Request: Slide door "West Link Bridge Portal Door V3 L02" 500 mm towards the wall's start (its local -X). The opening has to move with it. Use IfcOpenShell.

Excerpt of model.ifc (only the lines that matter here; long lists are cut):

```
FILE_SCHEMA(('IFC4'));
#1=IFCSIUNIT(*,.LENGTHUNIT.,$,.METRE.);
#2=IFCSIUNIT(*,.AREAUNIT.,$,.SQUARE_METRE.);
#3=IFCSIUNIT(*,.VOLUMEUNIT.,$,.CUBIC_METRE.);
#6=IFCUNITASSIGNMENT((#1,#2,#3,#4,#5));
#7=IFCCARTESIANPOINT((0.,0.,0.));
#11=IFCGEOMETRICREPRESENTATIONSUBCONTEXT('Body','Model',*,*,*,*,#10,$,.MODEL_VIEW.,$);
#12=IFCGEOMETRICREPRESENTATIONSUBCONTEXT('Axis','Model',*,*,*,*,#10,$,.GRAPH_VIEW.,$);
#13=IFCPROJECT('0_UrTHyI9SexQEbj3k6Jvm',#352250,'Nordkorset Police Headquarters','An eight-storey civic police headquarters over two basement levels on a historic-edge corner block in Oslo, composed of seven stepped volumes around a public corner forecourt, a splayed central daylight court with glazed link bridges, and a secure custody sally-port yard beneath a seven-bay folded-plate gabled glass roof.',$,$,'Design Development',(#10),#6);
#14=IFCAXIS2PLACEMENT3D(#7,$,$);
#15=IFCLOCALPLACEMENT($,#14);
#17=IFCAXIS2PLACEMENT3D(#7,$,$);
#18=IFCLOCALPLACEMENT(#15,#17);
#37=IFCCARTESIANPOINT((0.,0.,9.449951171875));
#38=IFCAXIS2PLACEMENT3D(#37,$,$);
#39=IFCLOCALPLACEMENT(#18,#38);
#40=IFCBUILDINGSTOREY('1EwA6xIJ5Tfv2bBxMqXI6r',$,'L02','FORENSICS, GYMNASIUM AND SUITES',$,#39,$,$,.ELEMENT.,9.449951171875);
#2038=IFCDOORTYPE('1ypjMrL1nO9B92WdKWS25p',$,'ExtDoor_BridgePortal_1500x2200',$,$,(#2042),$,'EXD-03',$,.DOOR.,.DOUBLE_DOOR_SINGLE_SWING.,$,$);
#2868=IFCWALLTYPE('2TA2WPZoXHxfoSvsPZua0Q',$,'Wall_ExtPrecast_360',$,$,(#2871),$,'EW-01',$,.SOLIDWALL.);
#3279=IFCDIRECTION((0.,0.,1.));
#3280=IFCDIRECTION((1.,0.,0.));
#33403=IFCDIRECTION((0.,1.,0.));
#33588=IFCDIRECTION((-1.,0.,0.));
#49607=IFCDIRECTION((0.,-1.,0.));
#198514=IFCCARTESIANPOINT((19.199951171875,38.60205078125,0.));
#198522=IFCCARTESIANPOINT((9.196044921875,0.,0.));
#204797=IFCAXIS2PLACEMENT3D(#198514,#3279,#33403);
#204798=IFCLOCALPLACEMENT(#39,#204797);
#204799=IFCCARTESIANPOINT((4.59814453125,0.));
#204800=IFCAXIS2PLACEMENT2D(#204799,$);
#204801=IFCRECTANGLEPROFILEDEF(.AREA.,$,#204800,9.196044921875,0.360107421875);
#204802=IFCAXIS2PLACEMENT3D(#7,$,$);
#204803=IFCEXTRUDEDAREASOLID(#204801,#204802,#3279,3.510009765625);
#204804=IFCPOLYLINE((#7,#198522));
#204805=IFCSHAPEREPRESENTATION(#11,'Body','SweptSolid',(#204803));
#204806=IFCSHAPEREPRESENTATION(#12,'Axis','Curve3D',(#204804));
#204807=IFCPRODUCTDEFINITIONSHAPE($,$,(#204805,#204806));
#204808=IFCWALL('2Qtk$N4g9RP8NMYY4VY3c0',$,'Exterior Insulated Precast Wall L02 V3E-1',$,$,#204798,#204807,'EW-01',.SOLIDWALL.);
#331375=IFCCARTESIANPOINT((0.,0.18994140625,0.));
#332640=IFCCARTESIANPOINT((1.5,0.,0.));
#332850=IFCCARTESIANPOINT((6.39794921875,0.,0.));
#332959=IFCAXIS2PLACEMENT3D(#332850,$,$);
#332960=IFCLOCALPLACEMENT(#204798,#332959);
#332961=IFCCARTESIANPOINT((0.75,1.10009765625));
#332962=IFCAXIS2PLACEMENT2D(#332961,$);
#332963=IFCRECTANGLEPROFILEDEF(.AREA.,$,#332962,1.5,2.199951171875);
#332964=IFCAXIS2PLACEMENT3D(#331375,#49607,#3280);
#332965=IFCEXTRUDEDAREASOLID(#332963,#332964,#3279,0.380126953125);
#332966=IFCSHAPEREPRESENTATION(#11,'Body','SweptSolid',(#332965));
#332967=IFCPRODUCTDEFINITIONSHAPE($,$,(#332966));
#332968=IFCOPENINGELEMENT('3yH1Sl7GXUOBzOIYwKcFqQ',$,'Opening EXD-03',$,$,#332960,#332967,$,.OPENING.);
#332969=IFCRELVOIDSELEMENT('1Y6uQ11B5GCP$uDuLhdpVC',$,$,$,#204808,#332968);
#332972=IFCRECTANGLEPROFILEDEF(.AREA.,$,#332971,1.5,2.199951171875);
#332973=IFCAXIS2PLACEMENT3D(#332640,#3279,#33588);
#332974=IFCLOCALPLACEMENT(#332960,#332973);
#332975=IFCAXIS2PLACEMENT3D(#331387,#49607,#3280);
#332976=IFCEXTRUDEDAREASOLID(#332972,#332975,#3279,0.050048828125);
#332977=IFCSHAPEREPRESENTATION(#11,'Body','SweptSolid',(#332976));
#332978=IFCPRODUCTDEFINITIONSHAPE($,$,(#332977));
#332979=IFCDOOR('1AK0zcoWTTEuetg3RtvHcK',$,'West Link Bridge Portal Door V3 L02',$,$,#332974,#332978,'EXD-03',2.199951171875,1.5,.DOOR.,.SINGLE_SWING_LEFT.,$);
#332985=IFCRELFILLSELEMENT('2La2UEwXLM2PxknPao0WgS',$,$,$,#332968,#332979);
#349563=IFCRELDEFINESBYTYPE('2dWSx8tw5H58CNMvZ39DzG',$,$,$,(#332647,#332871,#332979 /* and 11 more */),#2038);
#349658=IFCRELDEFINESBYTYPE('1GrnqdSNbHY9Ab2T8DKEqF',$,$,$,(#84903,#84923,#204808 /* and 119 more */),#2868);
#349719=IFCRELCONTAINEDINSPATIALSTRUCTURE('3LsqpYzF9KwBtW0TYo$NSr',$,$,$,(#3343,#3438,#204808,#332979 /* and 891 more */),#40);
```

```python
import ifcopenshell
import ifcopenshell.api.geometry
import ifcopenshell.util.placement
import ifcopenshell.util.unit

model = ifcopenshell.open("model.ifc")
unit_scale = ifcopenshell.util.unit.calculate_unit_scale(model)

door = model.by_id(332979)
opening = door.FillsVoids[0].RelatingOpeningElement
wall = opening.VoidsElements[0].RelatingBuildingElement

wall_matrix = ifcopenshell.util.placement.get_local_placement(wall.ObjectPlacement)
shift = wall_matrix[:3, 0] * -0.5 / unit_scale
before = ifcopenshell.util.placement.get_local_placement(door.ObjectPlacement)[:3, 3].copy()

# The door is placed relative to its opening, so it follows when the opening moves.
matrix = ifcopenshell.util.placement.get_local_placement(opening.ObjectPlacement)
matrix[:3, 3] += shift
ifcopenshell.api.geometry.edit_object_placement(
    model, product=opening, matrix=matrix, is_si=False, should_transform_children=True
)

after = ifcopenshell.util.placement.get_local_placement(door.ObjectPlacement)[:3, 3]
print("door moved by", (after - before).round(3) + 0.0)

model.write("model_edited.ifc")
```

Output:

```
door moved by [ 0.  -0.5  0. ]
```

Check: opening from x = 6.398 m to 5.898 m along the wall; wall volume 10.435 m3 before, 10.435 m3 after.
